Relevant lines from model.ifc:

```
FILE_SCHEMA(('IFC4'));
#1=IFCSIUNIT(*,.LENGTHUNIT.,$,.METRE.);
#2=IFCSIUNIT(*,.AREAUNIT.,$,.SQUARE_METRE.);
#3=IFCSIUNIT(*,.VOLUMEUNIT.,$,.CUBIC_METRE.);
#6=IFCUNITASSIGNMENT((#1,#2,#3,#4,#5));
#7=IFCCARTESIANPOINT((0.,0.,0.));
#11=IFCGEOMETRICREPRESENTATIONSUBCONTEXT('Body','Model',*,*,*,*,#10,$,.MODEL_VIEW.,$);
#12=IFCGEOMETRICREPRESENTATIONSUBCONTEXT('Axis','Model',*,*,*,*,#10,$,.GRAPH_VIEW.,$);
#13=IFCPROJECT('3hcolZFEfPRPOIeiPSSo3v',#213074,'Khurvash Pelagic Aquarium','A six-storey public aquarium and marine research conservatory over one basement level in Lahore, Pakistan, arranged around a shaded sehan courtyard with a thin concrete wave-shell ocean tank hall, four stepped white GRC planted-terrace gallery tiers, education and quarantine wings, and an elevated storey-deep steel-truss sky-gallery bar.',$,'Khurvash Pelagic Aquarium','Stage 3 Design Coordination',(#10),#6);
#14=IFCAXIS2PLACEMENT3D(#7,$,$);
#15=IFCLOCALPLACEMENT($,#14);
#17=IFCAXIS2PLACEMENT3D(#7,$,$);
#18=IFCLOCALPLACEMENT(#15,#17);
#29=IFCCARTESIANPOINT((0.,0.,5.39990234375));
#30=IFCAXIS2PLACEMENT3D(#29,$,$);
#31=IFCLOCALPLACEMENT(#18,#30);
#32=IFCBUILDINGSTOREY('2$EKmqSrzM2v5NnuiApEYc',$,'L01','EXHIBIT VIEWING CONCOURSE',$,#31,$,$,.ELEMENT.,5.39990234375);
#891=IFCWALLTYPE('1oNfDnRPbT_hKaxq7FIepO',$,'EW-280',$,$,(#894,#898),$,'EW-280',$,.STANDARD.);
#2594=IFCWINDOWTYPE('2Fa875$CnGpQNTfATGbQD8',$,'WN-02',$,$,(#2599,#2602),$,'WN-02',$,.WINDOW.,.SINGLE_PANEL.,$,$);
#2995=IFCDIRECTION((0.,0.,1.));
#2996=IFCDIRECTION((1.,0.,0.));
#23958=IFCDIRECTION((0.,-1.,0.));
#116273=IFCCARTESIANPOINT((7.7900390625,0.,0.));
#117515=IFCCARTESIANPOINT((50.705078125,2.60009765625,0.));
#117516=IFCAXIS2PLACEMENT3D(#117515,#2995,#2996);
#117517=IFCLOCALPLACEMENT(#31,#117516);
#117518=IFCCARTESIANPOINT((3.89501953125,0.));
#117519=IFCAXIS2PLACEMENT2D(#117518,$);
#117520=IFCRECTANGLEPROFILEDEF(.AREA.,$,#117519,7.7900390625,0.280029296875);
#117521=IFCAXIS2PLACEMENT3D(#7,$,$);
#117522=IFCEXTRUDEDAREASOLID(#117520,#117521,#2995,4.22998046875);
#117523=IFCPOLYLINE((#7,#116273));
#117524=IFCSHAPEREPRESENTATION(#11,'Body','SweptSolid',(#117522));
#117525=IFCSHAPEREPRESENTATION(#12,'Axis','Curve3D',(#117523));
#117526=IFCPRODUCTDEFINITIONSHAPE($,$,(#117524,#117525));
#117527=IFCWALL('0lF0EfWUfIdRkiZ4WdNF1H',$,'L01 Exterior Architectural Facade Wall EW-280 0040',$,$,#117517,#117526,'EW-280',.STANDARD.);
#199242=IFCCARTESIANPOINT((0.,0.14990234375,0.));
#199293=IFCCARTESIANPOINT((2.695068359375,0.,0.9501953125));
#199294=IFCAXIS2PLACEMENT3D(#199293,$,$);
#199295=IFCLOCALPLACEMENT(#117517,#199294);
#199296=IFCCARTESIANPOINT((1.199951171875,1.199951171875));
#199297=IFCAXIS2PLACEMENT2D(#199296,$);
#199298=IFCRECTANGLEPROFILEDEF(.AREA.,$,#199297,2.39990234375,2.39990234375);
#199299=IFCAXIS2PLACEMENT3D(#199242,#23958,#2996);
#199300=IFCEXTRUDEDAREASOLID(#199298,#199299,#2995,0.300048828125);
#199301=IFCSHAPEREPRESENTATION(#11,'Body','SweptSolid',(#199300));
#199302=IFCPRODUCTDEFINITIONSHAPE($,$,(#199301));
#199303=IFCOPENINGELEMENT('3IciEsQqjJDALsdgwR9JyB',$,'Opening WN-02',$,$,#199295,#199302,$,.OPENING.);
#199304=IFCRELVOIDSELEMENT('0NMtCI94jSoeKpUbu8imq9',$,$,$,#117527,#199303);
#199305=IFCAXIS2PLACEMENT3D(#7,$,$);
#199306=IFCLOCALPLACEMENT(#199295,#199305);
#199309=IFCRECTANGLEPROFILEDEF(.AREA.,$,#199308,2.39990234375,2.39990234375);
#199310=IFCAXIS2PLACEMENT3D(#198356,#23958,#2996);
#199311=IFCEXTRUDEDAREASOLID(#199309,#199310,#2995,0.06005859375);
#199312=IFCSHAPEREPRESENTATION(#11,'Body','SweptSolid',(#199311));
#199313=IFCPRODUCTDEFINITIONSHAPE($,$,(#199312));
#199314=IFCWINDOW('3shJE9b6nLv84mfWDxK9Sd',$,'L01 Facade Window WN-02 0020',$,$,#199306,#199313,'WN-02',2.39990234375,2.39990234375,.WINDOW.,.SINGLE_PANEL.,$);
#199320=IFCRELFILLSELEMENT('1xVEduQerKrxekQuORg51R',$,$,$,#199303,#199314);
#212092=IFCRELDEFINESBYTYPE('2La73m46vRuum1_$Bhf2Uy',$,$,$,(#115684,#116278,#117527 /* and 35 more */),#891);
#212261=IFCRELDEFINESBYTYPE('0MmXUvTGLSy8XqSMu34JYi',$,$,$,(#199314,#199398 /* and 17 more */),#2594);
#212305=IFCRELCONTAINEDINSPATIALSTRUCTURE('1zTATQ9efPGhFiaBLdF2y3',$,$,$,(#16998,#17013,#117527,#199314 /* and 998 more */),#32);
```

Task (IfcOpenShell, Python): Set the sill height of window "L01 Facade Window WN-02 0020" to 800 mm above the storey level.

```python
import numpy as np
import ifcopenshell
import ifcopenshell.api.geometry
import ifcopenshell.geom
import ifcopenshell.util.element
import ifcopenshell.util.placement
import ifcopenshell.util.shape
import ifcopenshell.util.unit

model = ifcopenshell.open("model.ifc")
unit_scale = ifcopenshell.util.unit.calculate_unit_scale(model)

window = model.by_guid("3shJE9b6nLv84mfWDxK9Sd")
opening = window.FillsVoids[0].RelatingOpeningElement
storey = ifcopenshell.util.element.get_container(window, ifc_class="IfcBuildingStorey")
level = ifcopenshell.util.placement.get_local_placement(storey.ObjectPlacement)[2, 3]

# The opening's origin need not be at the sill, so measure its lowest point.
shape = ifcopenshell.geom.create_shape(ifcopenshell.geom.settings(), opening)
bottom = ifcopenshell.util.shape.get_shape_bottom_elevation(shape, shape.geometry) / unit_scale
dz = level + 0.8 / unit_scale - bottom

shift = np.array([0.0, 0.0, dz])
# The window is placed relative to its opening, so it follows when the opening moves.
matrix = ifcopenshell.util.placement.get_local_placement(opening.ObjectPlacement)
matrix[:3, 3] += shift
ifcopenshell.api.geometry.edit_object_placement(
    model, product=opening, matrix=matrix, is_si=False, should_transform_children=True
)

print(f"moved by {dz * unit_scale:+.3f} m")

model.write("model-out.ifc")
```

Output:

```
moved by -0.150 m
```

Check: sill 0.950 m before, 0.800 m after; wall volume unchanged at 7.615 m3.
